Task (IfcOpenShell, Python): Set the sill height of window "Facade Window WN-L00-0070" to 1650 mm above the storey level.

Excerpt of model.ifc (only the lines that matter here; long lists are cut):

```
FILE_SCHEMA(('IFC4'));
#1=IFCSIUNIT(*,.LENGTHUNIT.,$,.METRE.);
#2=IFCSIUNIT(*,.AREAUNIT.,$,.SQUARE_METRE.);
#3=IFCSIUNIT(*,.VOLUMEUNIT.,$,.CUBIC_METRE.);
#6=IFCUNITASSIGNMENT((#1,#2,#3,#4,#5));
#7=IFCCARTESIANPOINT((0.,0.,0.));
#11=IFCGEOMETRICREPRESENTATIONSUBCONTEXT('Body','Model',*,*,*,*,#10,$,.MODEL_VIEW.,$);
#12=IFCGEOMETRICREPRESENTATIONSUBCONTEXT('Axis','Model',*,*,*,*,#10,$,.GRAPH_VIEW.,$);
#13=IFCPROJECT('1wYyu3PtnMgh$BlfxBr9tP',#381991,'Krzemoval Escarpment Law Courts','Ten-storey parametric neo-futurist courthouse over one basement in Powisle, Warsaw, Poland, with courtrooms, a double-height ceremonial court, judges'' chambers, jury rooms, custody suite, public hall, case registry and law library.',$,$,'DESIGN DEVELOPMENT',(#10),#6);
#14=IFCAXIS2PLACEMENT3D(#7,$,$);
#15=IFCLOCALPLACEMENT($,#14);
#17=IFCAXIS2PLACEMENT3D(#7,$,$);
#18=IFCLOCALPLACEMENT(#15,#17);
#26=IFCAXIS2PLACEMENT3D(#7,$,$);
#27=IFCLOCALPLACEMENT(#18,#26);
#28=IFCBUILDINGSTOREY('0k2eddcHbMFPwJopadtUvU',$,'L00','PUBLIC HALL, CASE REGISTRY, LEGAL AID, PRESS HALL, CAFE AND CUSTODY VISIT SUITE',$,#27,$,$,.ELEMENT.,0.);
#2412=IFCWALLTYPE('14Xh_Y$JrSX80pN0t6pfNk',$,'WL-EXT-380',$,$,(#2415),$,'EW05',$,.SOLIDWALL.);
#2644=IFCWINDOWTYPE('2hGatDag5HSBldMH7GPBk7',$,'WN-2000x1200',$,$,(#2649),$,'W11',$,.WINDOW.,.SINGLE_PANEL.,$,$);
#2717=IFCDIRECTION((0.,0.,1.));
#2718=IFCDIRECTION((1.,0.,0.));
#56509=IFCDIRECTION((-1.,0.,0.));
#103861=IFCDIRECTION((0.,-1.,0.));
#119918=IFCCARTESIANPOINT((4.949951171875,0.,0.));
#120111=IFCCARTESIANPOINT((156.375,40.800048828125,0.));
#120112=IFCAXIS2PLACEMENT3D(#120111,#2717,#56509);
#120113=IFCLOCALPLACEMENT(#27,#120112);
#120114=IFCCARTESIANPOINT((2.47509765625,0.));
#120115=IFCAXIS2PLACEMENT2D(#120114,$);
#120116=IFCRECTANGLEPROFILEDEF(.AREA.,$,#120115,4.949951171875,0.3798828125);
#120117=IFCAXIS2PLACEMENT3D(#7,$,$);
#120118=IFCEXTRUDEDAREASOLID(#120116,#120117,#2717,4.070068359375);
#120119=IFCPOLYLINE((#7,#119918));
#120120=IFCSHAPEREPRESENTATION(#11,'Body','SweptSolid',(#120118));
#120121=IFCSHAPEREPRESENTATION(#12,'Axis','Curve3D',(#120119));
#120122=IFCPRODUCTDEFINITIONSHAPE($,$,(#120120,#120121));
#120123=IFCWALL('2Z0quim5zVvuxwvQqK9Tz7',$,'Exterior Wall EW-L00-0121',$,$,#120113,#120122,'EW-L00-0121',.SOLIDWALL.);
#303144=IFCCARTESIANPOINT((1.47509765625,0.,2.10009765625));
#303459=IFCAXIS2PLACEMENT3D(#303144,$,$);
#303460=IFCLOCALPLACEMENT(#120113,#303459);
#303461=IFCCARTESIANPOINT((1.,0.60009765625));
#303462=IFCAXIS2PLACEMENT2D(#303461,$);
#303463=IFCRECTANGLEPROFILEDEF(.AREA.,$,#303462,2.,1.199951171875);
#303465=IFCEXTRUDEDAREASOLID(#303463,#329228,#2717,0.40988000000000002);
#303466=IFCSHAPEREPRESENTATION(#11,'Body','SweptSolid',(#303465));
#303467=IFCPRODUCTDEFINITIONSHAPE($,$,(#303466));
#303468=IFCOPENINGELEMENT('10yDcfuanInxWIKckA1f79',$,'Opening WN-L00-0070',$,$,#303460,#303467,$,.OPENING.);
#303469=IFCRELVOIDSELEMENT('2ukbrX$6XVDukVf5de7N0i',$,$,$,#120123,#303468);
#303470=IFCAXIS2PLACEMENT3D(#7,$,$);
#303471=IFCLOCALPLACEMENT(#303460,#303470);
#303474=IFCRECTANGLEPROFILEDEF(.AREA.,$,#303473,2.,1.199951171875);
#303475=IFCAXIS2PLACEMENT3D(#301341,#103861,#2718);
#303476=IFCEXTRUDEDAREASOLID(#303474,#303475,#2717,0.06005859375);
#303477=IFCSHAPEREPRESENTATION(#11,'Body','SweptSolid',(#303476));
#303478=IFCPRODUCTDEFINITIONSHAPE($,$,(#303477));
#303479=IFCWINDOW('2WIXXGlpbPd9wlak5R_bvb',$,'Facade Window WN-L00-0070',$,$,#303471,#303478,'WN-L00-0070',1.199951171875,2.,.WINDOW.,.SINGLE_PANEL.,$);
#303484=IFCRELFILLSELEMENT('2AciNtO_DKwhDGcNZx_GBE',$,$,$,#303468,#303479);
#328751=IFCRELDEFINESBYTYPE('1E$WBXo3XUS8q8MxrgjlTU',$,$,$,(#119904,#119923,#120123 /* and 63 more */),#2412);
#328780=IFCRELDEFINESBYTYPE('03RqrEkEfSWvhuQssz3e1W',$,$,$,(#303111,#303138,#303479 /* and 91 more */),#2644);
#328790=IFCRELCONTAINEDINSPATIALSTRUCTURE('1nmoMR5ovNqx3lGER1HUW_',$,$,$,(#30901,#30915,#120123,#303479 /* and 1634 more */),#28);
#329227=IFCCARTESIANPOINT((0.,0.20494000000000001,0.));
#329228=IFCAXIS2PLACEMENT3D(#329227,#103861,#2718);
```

```python
import numpy as np
import ifcopenshell
import ifcopenshell.api.geometry
import ifcopenshell.geom
import ifcopenshell.util.element
import ifcopenshell.util.placement
import ifcopenshell.util.shape
import ifcopenshell.util.unit

model = ifcopenshell.open("model.ifc")
unit_scale = ifcopenshell.util.unit.calculate_unit_scale(model)

window = model.by_guid("2WIXXGlpbPd9wlak5R_bvb")
opening = window.FillsVoids[0].RelatingOpeningElement
storey = ifcopenshell.util.element.get_container(window, ifc_class="IfcBuildingStorey")
level = ifcopenshell.util.placement.get_local_placement(storey.ObjectPlacement)[2, 3]

# The opening's origin need not be at the sill, so measure its lowest point.
shape = ifcopenshell.geom.create_shape(ifcopenshell.geom.settings(), opening)
bottom = ifcopenshell.util.shape.get_shape_bottom_elevation(shape, shape.geometry) / unit_scale
dz = level + 1.65 - bottom

shift = np.array([0.0, 0.0, dz])
# The window is placed relative to its opening, so it follows when the opening moves.
matrix = ifcopenshell.util.placement.get_local_placement(opening.ObjectPlacement)
matrix[:3, 3] += shift
ifcopenshell.api.geometry.edit_object_placement(
    model, product=opening, matrix=matrix, is_si=False, should_transform_children=True
)

print(f"moved by {dz * unit_scale:+.3f} m")

model.write("model_v2.ifc")
```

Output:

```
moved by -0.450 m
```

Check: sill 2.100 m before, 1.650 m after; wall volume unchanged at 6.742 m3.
